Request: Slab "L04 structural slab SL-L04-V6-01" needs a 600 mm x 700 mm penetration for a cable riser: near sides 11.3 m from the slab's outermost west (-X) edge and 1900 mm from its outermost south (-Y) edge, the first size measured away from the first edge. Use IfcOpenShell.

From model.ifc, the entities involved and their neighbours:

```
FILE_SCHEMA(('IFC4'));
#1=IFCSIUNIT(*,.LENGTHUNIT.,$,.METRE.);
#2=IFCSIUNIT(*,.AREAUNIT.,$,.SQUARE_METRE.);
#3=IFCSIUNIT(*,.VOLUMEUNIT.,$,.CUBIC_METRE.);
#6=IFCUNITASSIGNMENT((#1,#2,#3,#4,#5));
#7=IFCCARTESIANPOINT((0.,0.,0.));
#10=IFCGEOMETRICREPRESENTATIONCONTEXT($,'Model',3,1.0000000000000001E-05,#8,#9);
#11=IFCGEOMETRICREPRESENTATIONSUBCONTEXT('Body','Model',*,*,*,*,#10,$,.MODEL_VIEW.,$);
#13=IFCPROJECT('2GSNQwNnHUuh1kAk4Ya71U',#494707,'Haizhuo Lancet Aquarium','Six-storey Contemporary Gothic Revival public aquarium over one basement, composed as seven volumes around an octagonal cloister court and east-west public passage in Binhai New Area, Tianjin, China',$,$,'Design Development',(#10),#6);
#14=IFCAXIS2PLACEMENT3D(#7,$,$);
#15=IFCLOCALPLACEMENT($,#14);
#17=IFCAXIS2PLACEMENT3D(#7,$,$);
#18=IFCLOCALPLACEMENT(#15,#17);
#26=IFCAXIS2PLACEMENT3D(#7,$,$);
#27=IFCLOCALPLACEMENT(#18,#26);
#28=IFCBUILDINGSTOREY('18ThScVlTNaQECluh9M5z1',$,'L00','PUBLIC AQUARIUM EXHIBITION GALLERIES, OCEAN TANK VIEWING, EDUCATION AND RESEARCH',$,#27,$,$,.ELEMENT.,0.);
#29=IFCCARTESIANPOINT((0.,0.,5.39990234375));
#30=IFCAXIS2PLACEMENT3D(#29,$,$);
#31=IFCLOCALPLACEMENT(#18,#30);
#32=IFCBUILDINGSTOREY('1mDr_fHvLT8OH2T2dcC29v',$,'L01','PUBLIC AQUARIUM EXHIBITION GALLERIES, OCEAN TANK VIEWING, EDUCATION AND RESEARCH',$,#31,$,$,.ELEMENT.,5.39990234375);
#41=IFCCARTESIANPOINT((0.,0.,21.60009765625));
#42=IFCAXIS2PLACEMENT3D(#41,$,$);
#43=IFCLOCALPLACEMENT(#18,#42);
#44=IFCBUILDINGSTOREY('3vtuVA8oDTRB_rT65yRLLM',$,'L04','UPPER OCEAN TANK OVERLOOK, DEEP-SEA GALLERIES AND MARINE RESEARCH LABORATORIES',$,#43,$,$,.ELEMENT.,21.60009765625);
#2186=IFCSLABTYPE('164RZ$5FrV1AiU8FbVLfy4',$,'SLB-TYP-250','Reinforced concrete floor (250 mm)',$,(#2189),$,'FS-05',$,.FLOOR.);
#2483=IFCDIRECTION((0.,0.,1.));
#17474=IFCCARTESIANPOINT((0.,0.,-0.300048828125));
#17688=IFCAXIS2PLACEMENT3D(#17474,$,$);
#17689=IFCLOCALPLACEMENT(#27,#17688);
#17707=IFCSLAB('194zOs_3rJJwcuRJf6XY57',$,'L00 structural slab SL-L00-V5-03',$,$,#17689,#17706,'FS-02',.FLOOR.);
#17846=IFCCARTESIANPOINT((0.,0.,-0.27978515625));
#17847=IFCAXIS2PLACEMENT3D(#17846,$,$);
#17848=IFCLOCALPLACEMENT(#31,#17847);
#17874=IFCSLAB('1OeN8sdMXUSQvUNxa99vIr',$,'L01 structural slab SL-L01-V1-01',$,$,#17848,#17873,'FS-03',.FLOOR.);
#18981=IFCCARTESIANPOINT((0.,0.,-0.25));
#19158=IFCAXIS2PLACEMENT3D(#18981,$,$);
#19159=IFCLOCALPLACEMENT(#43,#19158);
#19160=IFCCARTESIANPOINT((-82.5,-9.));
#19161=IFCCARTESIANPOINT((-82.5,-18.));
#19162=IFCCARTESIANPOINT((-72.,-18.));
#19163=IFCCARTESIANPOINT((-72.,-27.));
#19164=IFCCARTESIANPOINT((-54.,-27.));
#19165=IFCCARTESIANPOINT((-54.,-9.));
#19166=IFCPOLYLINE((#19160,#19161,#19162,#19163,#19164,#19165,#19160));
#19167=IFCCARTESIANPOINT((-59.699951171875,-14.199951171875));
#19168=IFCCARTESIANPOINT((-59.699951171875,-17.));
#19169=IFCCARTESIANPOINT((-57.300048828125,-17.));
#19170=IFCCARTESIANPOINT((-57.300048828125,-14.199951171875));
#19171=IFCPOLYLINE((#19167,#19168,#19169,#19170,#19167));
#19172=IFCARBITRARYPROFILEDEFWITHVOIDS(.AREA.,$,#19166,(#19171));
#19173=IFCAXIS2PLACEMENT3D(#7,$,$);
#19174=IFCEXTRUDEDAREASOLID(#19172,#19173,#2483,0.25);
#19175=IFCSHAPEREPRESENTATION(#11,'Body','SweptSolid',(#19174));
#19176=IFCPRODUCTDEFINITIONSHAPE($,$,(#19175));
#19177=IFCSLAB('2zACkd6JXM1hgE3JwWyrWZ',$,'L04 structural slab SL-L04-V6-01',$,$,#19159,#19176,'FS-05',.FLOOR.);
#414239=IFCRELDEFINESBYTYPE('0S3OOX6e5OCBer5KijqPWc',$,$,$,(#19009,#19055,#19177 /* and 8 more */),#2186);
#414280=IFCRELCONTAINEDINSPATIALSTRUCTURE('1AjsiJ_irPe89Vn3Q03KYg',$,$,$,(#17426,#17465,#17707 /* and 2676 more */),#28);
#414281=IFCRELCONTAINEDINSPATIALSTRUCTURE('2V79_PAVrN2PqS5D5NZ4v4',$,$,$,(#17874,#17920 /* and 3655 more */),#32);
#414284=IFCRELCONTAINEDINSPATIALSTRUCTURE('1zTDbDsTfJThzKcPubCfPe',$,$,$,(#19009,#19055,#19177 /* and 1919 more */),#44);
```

```python
import numpy as np
import ifcopenshell
import ifcopenshell.api.feature
import ifcopenshell.api.geometry
import ifcopenshell.api.root
import ifcopenshell.geom
import ifcopenshell.util.placement
import ifcopenshell.util.representation
import ifcopenshell.util.shape
import ifcopenshell.util.unit

model = ifcopenshell.open("model.ifc")
unit_scale = ifcopenshell.util.unit.calculate_unit_scale(model)
settings = ifcopenshell.geom.settings()


def volume(element):
    """Net volume in cubic metres, openings subtracted."""
    shape = ifcopenshell.geom.create_shape(settings, element)
    return ifcopenshell.util.shape.get_volume(shape.geometry)


slab = model.by_guid("2zACkd6JXM1hgE3JwWyrWZ")
before = volume(slab)

# Extent in the slab's own axes, in metres. The edges named are its -X and -Y sides.
slab_shape = ifcopenshell.geom.create_shape(settings, slab)
vertices = ifcopenshell.util.shape.get_vertices(slab_shape.geometry)
x_min, y_min, bottom = vertices.min(axis=0)
top = vertices[:, 2].max()

opening = ifcopenshell.api.root.create_entity(model, ifc_class="IfcOpeningElement", name="Cable riser opening", predefined_type="OPENING")
context = ifcopenshell.util.representation.get_context(model, "Model", "Body", "MODEL_VIEW")
width, depth = 0.6, 0.7
outline = [(0.0, 0.0), (width, 0.0), (width, depth), (0.0, depth), (0.0, 0.0)]
# Overshoot both faces by 50 mm so the cut is clean.
shape = ifcopenshell.api.geometry.add_slab_representation(
    model, context=context, depth=top - bottom + 0.1, polyline=outline
)
ifcopenshell.api.geometry.assign_representation(model, product=opening, representation=shape)

matrix = ifcopenshell.util.placement.get_local_placement(slab.ObjectPlacement)
matrix[:, 3] = matrix @ np.append(np.array([x_min + 11.3, y_min + 1.9, bottom - 0.05]) / unit_scale, 1.0)
ifcopenshell.api.geometry.edit_object_placement(model, product=opening, matrix=matrix, is_si=False)
ifcopenshell.api.feature.add_feature(model, feature=opening, element=slab)

after = volume(slab)

print(f"slab volume {before:.3f} -> {after:.3f} m3")

model.write("model_v2.ifc")
```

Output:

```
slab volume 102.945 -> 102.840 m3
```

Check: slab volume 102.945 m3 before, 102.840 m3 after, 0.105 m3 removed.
